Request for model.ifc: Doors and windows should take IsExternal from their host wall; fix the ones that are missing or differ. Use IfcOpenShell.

First a look at what the model holds.

```python
import ifcopenshell
import ifcopenshell.util.element

model = ifcopenshell.open("model.ifc")
print(model.schema)
seen = {}
for e in model.by_type("IfcDoor") + model.by_type("IfcWindow"):
    if not e.FillsVoids:
        continue
    host = e.FillsVoids[0].RelatingOpeningElement.VoidsElements[0].RelatingBuildingElement
    own = ifcopenshell.util.element.get_pset(e, f"Pset_{e.is_a()[3:].removesuffix('StandardCase')}Common", "IsExternal")
    wall = ifcopenshell.util.element.get_pset(host, "Pset_WallCommon", "IsExternal")
    seen[e.is_a(), own, wall] = seen.get((e.is_a(), own, wall), 0) + 1
for (cls, own, wall), count in sorted(seen.items(), key=str):
    print(count, cls, "IsExternal:", own, "| host wall:", wall)
```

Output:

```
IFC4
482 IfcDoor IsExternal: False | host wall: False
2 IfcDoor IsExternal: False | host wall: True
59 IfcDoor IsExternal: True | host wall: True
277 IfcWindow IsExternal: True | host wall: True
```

```python
import ifcopenshell
import ifcopenshell.api.pset
import ifcopenshell.util.element

model = ifcopenshell.open("model.ifc")

count = 0
for ifc_class, pset_name in (("IfcDoor", "Pset_DoorCommon"), ("IfcWindow", "Pset_WindowCommon")):
    for e in model.by_type(ifc_class):
        if not e.FillsVoids:
            continue
        host = e.FillsVoids[0].RelatingOpeningElement.VoidsElements[0].RelatingBuildingElement
        external = ifcopenshell.util.element.get_pset(host, "Pset_WallCommon", "IsExternal")
        if external is None or ifcopenshell.util.element.get_pset(e, pset_name, "IsExternal") == external:
            continue
        pset = ifcopenshell.api.pset.add_pset(model, product=e, name=pset_name)
        ifcopenshell.api.pset.edit_pset(model, pset=pset, properties={"IsExternal": external})
        count += 1

print(count, "updated")

model.write("model_rev.ifc")
```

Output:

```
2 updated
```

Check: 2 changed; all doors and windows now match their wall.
